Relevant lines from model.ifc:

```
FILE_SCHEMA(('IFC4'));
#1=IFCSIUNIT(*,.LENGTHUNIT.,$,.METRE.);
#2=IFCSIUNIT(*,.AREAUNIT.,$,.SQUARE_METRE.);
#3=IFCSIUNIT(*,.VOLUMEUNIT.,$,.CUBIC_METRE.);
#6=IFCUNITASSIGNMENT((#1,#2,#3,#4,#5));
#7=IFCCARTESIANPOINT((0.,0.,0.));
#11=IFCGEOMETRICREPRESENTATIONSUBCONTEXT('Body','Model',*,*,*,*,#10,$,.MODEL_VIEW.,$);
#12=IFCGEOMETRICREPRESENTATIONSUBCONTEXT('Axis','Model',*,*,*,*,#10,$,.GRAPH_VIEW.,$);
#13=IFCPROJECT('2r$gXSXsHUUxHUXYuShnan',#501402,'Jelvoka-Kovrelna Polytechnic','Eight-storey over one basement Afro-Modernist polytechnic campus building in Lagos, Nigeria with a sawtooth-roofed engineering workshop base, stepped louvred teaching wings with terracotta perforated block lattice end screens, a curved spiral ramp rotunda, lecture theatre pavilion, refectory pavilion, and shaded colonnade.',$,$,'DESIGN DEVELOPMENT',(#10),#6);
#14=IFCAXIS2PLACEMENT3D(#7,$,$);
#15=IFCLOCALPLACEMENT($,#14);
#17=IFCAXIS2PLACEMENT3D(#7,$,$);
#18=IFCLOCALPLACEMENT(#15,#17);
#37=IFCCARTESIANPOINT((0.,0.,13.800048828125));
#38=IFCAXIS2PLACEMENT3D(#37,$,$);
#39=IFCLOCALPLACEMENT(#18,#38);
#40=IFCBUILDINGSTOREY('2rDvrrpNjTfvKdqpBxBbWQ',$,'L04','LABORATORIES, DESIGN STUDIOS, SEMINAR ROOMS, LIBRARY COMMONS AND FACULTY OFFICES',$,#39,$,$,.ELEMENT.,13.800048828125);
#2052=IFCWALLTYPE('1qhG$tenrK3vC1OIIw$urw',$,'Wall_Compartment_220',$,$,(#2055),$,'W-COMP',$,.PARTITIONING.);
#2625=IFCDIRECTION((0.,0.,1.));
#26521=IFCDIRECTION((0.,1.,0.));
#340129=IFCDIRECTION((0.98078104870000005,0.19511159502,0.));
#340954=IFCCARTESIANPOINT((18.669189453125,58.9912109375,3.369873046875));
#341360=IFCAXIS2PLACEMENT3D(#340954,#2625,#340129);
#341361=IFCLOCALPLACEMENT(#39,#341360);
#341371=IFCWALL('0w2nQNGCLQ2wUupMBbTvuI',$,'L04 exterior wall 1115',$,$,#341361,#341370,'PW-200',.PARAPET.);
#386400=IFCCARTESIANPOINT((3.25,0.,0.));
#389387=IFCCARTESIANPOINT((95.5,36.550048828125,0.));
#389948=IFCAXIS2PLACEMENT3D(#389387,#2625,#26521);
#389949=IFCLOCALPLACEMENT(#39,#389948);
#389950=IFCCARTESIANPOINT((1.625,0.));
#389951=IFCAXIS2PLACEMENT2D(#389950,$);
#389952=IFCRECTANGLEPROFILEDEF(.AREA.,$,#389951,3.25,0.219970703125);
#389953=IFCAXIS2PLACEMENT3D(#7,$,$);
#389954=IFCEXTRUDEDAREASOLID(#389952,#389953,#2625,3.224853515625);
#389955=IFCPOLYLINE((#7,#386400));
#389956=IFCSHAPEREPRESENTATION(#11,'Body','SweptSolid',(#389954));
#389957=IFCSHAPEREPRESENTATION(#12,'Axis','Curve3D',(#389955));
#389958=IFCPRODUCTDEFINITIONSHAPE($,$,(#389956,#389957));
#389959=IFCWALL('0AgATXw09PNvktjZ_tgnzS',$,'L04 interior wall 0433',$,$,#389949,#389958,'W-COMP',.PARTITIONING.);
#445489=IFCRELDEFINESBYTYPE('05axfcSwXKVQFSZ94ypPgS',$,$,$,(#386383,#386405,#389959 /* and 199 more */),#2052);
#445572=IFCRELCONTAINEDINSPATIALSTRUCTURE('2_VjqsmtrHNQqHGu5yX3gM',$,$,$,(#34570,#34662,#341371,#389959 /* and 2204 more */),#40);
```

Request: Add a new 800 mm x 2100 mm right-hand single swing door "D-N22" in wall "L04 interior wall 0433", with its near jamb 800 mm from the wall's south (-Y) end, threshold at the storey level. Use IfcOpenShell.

```python
import numpy as np
import ifcopenshell
import ifcopenshell.api.feature
import ifcopenshell.api.geometry
import ifcopenshell.api.root
import ifcopenshell.api.spatial
import ifcopenshell.geom
import ifcopenshell.util.element
import ifcopenshell.util.placement
import ifcopenshell.util.representation
import ifcopenshell.util.shape
import ifcopenshell.util.unit

model = ifcopenshell.open("model.ifc")
unit_scale = ifcopenshell.util.unit.calculate_unit_scale(model)
settings = ifcopenshell.geom.settings()


def volume(element):
    """Net volume in cubic metres, openings subtracted."""
    shape = ifcopenshell.geom.create_shape(settings, element)
    return ifcopenshell.util.shape.get_volume(shape.geometry)


wall = model.by_guid("0AgATXw09PNvktjZ_tgnzS")
storey = ifcopenshell.util.element.get_container(wall, ifc_class="IfcBuildingStorey")
context = ifcopenshell.util.representation.get_context(model, "Model", "Body", "MODEL_VIEW")
before = volume(wall)

width, height, from_end, sill = 0.8, 2.1, 0.8, 0.0  # metres

# The wall runs along its own X axis, and the end named is its -X end.
wall_shape = ifcopenshell.geom.create_shape(settings, wall)
x, y, z = ifcopenshell.util.shape.get_vertices(wall_shape.geometry).T
start = x.min() + from_end
face, thickness = float(y.min()), float(y.max() - y.min())
wall_matrix = ifcopenshell.util.placement.get_local_placement(wall.ObjectPlacement)
level = ifcopenshell.util.placement.get_local_placement(storey.ObjectPlacement)[2, 3]


def in_wall(x, y):
    """Placement at x, y metres in the wall's axes, at sill height."""
    matrix = wall_matrix.copy()
    matrix[:, 3] = wall_matrix @ np.array([x / unit_scale, y / unit_scale, 0.0, 1.0])
    matrix[2, 3] = level + sill / unit_scale
    return matrix


# Opening: a box that overshoots both wall faces by 50 mm.
opening = ifcopenshell.api.root.create_entity(model, ifc_class="IfcOpeningElement", predefined_type="OPENING")
box = ifcopenshell.api.geometry.add_wall_representation(
    model, context=context, length=width, height=height, thickness=thickness + 0.1
)
ifcopenshell.api.geometry.assign_representation(model, product=opening, representation=box)
ifcopenshell.api.geometry.edit_object_placement(model, product=opening, matrix=in_wall(start, face - 0.05), is_si=False)
ifcopenshell.api.feature.add_feature(model, feature=opening, element=wall)

door = ifcopenshell.api.root.create_entity(model, ifc_class="IfcDoor", name="D-N22", predefined_type="DOOR")
door.OverallWidth, door.OverallHeight = width / unit_scale, height / unit_scale
door.OperationType = "SINGLE_SWING_RIGHT"
body = ifcopenshell.api.geometry.add_door_representation(
    model,
    context=context,
    overall_width=door.OverallWidth,
    overall_height=door.OverallHeight,
    operation_type="SINGLE_SWING_RIGHT",
    lining_properties={"LiningDepth": thickness / unit_scale, "ThresholdDepth": thickness / unit_scale},
)
ifcopenshell.api.geometry.assign_representation(model, product=door, representation=body)
ifcopenshell.api.spatial.assign_container(model, products=[door], relating_structure=storey)
ifcopenshell.api.feature.add_filling(model, opening=opening, element=door)

# The lining spans the wall, so the door starts at the wall face.
ifcopenshell.api.geometry.edit_object_placement(model, product=door, matrix=in_wall(start, face), is_si=False)

after = volume(wall)

print(f"wall volume {before:.3f} -> {after:.3f} m3")

model.write("model_rev.ifc")
```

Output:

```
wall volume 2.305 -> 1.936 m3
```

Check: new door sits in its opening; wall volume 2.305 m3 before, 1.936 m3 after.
